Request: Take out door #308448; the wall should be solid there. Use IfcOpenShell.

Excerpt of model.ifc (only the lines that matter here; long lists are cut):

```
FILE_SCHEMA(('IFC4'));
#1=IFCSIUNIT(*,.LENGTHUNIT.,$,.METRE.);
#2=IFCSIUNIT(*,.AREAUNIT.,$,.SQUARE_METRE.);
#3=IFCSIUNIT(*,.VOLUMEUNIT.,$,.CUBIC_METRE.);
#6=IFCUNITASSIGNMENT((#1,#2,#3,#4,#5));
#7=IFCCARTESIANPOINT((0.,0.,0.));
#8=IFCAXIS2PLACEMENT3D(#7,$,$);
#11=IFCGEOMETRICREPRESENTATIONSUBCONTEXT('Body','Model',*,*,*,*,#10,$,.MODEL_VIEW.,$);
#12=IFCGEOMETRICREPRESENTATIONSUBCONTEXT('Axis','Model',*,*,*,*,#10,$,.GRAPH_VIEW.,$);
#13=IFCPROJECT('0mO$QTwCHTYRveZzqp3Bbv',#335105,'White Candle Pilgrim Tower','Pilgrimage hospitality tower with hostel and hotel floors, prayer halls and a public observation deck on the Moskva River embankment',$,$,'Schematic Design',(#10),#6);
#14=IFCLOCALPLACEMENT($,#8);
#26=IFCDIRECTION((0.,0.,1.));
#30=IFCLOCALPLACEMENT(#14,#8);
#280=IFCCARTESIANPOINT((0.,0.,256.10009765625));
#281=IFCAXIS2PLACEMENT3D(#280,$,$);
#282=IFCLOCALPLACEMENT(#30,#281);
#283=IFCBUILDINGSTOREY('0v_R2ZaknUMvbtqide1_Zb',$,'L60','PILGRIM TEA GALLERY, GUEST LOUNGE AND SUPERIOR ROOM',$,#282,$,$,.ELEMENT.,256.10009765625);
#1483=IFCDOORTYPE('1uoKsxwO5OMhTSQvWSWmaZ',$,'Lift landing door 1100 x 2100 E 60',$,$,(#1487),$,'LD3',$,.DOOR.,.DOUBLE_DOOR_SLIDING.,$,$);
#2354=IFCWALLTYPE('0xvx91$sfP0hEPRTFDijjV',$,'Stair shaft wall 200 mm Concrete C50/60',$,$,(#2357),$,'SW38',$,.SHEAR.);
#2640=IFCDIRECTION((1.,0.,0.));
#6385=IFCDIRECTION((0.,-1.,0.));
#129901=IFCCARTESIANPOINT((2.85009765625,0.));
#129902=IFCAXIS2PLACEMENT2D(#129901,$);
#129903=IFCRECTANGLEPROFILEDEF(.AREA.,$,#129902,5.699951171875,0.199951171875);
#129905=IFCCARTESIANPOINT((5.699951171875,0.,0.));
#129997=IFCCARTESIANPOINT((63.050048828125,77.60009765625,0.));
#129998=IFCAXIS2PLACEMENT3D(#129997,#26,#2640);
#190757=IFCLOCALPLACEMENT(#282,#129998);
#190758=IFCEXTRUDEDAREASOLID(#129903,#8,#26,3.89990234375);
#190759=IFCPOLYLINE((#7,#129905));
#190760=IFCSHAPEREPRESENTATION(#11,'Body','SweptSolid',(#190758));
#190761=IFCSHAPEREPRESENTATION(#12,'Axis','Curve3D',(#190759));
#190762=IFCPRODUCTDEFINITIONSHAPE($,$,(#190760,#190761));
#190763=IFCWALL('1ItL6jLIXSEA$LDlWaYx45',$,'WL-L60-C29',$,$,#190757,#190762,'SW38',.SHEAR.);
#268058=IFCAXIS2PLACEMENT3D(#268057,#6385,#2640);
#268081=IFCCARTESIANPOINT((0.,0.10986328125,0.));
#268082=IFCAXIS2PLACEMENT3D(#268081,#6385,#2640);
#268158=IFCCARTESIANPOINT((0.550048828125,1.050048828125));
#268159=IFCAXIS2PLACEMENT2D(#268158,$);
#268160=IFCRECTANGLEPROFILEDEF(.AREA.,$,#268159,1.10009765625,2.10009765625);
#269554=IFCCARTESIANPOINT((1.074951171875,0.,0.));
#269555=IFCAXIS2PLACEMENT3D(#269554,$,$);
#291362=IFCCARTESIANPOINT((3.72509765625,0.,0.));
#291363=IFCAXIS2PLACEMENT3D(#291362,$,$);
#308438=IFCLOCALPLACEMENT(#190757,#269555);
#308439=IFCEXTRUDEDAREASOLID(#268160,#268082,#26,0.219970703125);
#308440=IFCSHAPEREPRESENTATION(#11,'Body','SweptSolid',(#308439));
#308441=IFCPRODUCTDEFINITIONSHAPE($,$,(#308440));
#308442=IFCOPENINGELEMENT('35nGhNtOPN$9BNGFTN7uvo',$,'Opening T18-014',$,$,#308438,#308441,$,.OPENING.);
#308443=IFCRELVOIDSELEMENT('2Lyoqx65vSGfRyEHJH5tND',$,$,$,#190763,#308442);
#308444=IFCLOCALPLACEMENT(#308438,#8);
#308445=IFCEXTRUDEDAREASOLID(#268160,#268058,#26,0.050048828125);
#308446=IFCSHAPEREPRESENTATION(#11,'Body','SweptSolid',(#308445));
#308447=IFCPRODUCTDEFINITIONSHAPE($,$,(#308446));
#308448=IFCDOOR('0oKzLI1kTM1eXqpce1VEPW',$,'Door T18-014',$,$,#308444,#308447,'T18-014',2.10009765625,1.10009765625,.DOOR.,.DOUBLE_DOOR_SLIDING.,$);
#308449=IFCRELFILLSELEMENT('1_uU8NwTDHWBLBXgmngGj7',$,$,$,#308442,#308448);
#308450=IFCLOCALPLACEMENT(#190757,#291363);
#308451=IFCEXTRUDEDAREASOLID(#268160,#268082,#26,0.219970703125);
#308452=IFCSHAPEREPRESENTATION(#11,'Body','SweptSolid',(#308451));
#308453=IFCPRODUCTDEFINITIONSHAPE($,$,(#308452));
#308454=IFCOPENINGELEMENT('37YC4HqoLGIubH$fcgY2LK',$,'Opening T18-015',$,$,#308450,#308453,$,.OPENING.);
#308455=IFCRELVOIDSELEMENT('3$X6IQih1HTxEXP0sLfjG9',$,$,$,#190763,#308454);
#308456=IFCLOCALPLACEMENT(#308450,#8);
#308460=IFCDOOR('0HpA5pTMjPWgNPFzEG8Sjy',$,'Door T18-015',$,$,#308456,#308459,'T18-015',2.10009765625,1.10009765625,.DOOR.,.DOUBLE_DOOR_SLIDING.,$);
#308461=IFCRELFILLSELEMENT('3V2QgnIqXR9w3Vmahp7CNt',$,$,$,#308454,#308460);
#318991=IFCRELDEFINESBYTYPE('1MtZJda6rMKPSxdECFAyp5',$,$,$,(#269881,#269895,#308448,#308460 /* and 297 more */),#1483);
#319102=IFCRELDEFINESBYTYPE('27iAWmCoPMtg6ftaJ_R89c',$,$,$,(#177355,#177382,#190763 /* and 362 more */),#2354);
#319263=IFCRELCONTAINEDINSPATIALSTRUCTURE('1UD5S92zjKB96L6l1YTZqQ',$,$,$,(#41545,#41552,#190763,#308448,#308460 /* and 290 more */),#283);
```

```python
import ifcopenshell
import ifcopenshell.api.feature
import ifcopenshell.api.root
import ifcopenshell.geom
import ifcopenshell.util.shape

model = ifcopenshell.open("model.ifc")
settings = ifcopenshell.geom.settings()


def volume(element):
    """Net volume in cubic metres, openings subtracted."""
    shape = ifcopenshell.geom.create_shape(settings, element)
    return ifcopenshell.util.shape.get_volume(shape.geometry)


door = model.by_id(308448)
opening = door.FillsVoids[0].RelatingOpeningElement
wall = opening.VoidsElements[0].RelatingBuildingElement
before = volume(wall)

ifcopenshell.api.root.remove_product(model, product=door)
ifcopenshell.api.feature.remove_feature(model, feature=opening)

after = volume(wall)

print(f"wall volume {before:.3f} -> {after:.3f} m3")

model.write("model-out.ifc")
```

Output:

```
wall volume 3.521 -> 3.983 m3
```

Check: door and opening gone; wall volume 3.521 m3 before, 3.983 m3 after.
